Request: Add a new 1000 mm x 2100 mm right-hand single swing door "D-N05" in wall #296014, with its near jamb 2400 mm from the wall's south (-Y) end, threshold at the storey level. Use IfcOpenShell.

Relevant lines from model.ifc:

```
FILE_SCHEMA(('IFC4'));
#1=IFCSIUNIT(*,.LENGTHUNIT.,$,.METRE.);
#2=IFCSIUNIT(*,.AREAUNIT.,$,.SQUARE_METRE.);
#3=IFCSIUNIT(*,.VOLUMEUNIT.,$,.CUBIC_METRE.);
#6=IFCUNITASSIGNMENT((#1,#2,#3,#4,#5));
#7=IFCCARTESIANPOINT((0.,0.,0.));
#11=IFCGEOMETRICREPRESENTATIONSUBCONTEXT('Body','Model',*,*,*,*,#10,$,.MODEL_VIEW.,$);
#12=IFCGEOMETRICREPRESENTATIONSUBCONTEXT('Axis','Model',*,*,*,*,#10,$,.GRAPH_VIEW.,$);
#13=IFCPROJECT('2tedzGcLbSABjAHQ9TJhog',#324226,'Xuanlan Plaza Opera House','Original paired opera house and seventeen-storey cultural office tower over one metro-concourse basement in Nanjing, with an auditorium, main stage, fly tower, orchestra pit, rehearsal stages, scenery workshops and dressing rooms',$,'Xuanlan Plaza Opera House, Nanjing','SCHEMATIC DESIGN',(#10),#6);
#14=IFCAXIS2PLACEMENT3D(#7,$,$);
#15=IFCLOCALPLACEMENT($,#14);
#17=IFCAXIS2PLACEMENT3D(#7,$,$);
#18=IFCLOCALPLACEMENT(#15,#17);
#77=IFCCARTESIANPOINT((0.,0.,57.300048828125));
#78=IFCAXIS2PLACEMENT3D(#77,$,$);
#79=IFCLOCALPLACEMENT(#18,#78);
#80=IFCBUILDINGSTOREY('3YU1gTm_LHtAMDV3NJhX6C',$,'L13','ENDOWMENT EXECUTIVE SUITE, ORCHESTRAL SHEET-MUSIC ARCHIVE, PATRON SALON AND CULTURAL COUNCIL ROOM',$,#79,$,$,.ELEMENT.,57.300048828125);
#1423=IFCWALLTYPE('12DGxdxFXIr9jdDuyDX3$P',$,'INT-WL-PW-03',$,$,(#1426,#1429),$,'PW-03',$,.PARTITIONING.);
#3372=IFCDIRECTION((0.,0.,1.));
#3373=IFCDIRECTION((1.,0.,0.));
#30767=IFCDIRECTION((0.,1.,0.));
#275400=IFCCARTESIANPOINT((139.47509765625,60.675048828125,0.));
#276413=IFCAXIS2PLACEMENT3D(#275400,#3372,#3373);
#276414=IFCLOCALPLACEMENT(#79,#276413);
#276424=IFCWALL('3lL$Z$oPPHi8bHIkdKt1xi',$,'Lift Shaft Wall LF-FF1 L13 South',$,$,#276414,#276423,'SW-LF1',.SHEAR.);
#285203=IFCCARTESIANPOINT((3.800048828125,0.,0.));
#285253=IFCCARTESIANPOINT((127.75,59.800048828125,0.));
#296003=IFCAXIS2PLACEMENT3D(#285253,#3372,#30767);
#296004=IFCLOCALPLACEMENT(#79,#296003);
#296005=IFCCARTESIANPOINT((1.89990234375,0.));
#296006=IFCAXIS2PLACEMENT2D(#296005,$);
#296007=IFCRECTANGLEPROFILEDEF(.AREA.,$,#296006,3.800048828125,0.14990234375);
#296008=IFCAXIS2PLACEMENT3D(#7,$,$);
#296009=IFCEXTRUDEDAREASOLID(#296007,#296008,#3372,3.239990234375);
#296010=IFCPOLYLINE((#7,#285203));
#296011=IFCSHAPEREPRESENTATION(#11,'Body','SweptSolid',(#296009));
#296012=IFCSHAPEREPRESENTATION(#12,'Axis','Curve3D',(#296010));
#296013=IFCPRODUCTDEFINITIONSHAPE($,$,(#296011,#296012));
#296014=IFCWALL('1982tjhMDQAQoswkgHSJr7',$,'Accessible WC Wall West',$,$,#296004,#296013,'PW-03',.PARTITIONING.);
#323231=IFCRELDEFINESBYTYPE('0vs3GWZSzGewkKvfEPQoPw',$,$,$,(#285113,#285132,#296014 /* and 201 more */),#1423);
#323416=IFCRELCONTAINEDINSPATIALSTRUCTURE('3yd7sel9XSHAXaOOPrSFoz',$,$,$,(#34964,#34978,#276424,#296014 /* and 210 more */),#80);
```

```python
import numpy as np
import ifcopenshell
import ifcopenshell.api.feature
import ifcopenshell.api.geometry
import ifcopenshell.api.root
import ifcopenshell.api.spatial
import ifcopenshell.geom
import ifcopenshell.util.element
import ifcopenshell.util.placement
import ifcopenshell.util.representation
import ifcopenshell.util.shape
import ifcopenshell.util.unit

model = ifcopenshell.open("model.ifc")
unit_scale = ifcopenshell.util.unit.calculate_unit_scale(model)
settings = ifcopenshell.geom.settings()


def volume(element):
    """Net volume in cubic metres, openings subtracted."""
    shape = ifcopenshell.geom.create_shape(settings, element)
    return ifcopenshell.util.shape.get_volume(shape.geometry)


wall = model.by_guid("1982tjhMDQAQoswkgHSJr7")
storey = ifcopenshell.util.element.get_container(wall, ifc_class="IfcBuildingStorey")
context = ifcopenshell.util.representation.get_context(model, "Model", "Body", "MODEL_VIEW")
before = volume(wall)

width, height, from_end, sill = 1, 2.1, 2.4, 0.0  # metres

# The wall runs along its own X axis, and the end named is its -X end.
wall_shape = ifcopenshell.geom.create_shape(settings, wall)
x, y, z = ifcopenshell.util.shape.get_vertices(wall_shape.geometry).T
start = x.min() + from_end
face, thickness = float(y.min()), float(y.max() - y.min())
wall_matrix = ifcopenshell.util.placement.get_local_placement(wall.ObjectPlacement)
level = ifcopenshell.util.placement.get_local_placement(storey.ObjectPlacement)[2, 3]


def in_wall(x, y):
    """Placement at x, y metres in the wall's axes, at sill height."""
    matrix = wall_matrix.copy()
    matrix[:, 3] = wall_matrix @ np.array([x / unit_scale, y / unit_scale, 0.0, 1.0])
    matrix[2, 3] = level + sill / unit_scale
    return matrix


# Opening: a box that overshoots both wall faces by 50 mm.
opening = ifcopenshell.api.root.create_entity(model, ifc_class="IfcOpeningElement", predefined_type="OPENING")
box = ifcopenshell.api.geometry.add_wall_representation(
    model, context=context, length=width, height=height, thickness=thickness + 0.1
)
ifcopenshell.api.geometry.assign_representation(model, product=opening, representation=box)
ifcopenshell.api.geometry.edit_object_placement(model, product=opening, matrix=in_wall(start, face - 0.05), is_si=False)
ifcopenshell.api.feature.add_feature(model, feature=opening, element=wall)

door = ifcopenshell.api.root.create_entity(model, ifc_class="IfcDoor", name="D-N05", predefined_type="DOOR")
door.OverallWidth, door.OverallHeight = width / unit_scale, height / unit_scale
door.OperationType = "SINGLE_SWING_RIGHT"
body = ifcopenshell.api.geometry.add_door_representation(
    model,
    context=context,
    overall_width=door.OverallWidth,
    overall_height=door.OverallHeight,
    operation_type="SINGLE_SWING_RIGHT",
    lining_properties={"LiningDepth": thickness / unit_scale, "ThresholdDepth": thickness / unit_scale},
)
ifcopenshell.api.geometry.assign_representation(model, product=door, representation=body)
ifcopenshell.api.spatial.assign_container(model, products=[door], relating_structure=storey)
ifcopenshell.api.feature.add_filling(model, opening=opening, element=door)

# The lining spans the wall, so the door starts at the wall face.
ifcopenshell.api.geometry.edit_object_placement(model, product=door, matrix=in_wall(start, face), is_si=False)

after = volume(wall)

print(f"wall volume {before:.3f} -> {after:.3f} m3")

model.write("model_edited.ifc")
```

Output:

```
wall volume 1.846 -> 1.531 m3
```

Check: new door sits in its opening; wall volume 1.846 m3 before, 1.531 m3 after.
